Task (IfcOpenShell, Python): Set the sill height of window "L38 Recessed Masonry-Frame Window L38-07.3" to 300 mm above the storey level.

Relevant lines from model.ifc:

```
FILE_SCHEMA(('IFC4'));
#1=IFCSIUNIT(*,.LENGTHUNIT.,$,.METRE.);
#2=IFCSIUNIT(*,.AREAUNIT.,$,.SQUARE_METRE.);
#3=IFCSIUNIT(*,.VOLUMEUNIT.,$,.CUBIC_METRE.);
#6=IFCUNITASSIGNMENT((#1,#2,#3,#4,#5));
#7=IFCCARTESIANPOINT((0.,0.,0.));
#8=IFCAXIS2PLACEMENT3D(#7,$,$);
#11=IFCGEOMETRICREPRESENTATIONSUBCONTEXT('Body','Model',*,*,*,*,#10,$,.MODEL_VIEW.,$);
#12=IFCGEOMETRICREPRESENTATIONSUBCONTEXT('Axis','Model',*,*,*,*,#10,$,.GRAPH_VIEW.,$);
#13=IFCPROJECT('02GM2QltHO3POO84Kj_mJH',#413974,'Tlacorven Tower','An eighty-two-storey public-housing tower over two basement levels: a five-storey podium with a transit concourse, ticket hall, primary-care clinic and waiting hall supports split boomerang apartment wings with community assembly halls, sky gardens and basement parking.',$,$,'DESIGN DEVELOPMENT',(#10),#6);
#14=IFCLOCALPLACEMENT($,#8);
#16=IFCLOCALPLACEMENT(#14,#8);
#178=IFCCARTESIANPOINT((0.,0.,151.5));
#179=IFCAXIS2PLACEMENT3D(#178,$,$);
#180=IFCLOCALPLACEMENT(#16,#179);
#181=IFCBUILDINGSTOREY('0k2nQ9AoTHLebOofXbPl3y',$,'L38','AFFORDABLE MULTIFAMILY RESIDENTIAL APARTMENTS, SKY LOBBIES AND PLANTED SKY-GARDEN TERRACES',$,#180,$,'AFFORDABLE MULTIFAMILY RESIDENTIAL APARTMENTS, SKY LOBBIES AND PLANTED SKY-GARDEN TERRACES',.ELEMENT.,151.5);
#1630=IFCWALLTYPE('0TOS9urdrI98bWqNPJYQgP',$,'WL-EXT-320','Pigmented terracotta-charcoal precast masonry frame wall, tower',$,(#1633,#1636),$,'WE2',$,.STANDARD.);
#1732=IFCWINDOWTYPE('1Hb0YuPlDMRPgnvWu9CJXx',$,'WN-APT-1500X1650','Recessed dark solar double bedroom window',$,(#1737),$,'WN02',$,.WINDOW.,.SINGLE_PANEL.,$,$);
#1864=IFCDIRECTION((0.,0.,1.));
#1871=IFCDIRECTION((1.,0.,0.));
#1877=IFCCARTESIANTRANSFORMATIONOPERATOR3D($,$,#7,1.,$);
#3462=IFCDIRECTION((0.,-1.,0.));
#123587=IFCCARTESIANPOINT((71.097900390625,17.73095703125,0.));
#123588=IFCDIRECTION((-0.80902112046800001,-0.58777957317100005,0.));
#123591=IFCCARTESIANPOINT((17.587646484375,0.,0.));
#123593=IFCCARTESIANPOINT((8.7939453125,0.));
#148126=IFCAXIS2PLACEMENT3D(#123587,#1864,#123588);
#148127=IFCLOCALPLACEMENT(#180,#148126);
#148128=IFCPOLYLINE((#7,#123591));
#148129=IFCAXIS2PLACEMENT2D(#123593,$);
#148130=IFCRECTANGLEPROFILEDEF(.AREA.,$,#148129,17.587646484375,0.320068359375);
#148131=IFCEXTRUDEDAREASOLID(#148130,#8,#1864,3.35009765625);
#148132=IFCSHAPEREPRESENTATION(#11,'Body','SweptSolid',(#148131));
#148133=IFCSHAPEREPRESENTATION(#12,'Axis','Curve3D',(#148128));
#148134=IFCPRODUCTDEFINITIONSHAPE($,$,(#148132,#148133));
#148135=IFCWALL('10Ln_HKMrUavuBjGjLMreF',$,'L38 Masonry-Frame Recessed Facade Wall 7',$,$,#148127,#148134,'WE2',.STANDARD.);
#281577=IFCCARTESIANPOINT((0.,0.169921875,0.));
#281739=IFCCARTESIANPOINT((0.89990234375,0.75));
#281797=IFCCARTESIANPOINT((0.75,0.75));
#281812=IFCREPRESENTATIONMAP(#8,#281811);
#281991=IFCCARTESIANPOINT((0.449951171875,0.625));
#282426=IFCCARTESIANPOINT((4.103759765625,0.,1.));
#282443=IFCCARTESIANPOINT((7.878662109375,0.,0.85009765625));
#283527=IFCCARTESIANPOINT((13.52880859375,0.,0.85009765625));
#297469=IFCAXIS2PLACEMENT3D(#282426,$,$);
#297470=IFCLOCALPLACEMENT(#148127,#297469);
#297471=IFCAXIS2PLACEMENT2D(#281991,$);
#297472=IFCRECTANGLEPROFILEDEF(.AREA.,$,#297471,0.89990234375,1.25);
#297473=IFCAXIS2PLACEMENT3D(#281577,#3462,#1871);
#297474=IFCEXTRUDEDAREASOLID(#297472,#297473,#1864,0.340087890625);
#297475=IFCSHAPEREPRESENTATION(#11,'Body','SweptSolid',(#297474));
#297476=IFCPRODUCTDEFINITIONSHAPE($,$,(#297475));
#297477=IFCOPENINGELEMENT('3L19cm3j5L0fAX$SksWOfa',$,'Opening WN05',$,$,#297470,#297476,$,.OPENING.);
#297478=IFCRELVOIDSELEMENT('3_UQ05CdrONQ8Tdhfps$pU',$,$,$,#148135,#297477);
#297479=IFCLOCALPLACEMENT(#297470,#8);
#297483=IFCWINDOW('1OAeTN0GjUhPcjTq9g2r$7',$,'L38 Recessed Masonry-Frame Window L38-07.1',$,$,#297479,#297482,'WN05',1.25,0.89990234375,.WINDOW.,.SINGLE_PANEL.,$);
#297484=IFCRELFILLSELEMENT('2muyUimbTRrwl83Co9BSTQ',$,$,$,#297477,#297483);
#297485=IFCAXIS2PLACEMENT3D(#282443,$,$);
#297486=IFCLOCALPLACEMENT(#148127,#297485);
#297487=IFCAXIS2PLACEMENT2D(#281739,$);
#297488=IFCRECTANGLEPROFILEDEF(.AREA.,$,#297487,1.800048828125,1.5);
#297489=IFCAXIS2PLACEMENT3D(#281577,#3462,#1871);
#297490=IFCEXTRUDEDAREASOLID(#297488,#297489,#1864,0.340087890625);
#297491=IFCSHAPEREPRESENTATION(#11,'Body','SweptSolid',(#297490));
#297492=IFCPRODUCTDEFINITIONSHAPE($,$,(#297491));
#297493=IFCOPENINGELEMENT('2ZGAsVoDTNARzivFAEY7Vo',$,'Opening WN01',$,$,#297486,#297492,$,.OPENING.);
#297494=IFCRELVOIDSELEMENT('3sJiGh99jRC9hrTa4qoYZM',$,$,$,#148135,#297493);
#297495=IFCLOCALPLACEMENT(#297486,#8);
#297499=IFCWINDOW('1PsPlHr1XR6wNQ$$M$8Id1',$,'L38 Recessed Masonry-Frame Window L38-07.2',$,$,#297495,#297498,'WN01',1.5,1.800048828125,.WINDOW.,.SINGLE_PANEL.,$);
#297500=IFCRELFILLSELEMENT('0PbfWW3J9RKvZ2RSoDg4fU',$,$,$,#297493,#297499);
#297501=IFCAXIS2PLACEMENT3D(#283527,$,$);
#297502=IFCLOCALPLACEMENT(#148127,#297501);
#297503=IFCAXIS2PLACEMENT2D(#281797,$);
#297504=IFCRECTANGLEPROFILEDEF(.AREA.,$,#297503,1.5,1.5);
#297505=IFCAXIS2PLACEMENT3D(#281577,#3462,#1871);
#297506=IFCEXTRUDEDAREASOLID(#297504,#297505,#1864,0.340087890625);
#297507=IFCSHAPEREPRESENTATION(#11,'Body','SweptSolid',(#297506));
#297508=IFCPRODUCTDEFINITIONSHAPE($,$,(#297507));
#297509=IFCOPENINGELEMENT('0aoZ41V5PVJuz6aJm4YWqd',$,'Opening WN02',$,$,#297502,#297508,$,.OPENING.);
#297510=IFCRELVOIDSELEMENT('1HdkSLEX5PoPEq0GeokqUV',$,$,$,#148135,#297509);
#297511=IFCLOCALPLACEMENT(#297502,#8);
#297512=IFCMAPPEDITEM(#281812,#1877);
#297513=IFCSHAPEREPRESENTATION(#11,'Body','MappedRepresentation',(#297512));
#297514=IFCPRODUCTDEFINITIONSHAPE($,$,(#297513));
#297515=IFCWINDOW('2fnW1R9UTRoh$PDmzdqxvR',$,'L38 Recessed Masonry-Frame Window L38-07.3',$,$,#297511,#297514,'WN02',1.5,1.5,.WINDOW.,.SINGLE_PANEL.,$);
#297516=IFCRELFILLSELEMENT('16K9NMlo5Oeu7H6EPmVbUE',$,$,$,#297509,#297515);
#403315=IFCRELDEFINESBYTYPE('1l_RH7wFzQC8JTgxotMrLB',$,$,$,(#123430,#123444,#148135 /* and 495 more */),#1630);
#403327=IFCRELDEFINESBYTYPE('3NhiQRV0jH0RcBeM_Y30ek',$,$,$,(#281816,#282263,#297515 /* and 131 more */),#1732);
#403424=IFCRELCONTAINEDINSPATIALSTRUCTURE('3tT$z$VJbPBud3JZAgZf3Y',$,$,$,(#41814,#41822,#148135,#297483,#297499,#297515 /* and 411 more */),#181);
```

```python
import numpy as np
import ifcopenshell
import ifcopenshell.api.geometry
import ifcopenshell.geom
import ifcopenshell.util.element
import ifcopenshell.util.placement
import ifcopenshell.util.shape
import ifcopenshell.util.unit

model = ifcopenshell.open("model.ifc")
unit_scale = ifcopenshell.util.unit.calculate_unit_scale(model)

window = model.by_guid("2fnW1R9UTRoh$PDmzdqxvR")
opening = window.FillsVoids[0].RelatingOpeningElement
storey = ifcopenshell.util.element.get_container(window, ifc_class="IfcBuildingStorey")
level = ifcopenshell.util.placement.get_local_placement(storey.ObjectPlacement)[2, 3]

# The opening's origin need not be at the sill, so measure its lowest point.
shape = ifcopenshell.geom.create_shape(ifcopenshell.geom.settings(), opening)
bottom = ifcopenshell.util.shape.get_shape_bottom_elevation(shape, shape.geometry) / unit_scale
dz = level + 0.3 / unit_scale - bottom

shift = np.array([0.0, 0.0, dz])
# The window is placed relative to its opening, so it follows when the opening moves.
matrix = ifcopenshell.util.placement.get_local_placement(opening.ObjectPlacement)
matrix[:3, 3] += shift
ifcopenshell.api.geometry.edit_object_placement(
    model, product=opening, matrix=matrix, is_si=False, should_transform_children=True
)

print(f"moved by {dz * unit_scale:+.3f} m")

model.write("model-out.ifc")
```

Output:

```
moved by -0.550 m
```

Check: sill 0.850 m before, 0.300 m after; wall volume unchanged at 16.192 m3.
